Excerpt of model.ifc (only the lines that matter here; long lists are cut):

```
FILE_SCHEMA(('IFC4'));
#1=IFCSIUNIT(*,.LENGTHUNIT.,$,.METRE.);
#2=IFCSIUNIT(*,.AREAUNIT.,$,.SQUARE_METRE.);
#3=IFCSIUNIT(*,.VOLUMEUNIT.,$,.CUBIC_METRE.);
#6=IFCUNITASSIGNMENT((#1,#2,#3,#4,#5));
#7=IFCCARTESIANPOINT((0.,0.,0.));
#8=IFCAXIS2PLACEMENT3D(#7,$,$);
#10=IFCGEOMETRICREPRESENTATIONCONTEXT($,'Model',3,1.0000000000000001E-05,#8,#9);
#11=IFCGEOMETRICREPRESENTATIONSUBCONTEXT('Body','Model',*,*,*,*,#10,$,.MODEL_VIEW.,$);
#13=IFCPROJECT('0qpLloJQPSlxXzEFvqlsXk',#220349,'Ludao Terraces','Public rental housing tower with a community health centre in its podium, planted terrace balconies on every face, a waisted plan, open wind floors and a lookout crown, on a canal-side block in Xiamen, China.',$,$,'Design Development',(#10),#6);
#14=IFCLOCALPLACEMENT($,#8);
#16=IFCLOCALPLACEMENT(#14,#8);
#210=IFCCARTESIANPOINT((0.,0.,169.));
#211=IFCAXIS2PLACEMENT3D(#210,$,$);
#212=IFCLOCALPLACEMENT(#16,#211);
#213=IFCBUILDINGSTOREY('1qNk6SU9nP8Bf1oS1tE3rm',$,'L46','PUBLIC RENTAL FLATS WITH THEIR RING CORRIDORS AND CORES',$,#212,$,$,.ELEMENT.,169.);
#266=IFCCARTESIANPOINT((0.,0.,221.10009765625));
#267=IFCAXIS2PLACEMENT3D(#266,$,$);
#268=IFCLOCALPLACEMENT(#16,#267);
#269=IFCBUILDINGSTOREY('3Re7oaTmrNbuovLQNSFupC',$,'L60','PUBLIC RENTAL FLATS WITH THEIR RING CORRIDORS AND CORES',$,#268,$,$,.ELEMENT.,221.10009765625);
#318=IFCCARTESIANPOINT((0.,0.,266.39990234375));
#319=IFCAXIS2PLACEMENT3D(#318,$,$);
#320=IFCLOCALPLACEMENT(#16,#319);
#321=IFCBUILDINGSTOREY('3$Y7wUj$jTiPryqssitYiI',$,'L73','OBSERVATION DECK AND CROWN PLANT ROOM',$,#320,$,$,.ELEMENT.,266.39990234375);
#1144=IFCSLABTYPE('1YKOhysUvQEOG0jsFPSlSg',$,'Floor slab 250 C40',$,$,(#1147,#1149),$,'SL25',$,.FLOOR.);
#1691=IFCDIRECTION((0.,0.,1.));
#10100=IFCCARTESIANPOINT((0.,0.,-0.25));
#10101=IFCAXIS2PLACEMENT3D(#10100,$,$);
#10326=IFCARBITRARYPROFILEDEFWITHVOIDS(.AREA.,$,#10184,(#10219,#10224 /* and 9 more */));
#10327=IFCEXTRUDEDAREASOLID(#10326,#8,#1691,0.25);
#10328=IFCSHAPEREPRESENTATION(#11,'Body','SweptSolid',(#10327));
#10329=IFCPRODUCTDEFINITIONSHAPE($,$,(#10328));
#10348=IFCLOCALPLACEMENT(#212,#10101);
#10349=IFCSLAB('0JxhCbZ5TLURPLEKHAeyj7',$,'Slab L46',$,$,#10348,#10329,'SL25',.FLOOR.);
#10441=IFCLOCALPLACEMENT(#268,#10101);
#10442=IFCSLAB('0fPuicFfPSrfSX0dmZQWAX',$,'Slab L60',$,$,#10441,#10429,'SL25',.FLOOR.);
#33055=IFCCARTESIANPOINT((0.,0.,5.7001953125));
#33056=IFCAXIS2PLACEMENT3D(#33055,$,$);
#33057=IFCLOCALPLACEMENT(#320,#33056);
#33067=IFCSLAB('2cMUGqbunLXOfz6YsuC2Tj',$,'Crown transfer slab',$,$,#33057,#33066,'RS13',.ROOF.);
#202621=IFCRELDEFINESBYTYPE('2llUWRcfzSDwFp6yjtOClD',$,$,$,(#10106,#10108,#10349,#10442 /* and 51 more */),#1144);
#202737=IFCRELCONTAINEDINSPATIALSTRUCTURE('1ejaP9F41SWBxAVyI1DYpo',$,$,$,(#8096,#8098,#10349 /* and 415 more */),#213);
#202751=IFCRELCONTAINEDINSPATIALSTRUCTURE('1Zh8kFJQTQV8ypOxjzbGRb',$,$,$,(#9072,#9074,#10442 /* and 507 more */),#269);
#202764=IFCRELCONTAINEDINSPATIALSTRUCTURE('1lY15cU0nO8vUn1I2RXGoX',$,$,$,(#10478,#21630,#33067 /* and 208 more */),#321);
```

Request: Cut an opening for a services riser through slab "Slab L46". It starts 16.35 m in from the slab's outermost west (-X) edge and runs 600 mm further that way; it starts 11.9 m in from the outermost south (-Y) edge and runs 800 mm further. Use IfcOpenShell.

```python
import numpy as np
import ifcopenshell
import ifcopenshell.api.feature
import ifcopenshell.api.geometry
import ifcopenshell.api.root
import ifcopenshell.geom
import ifcopenshell.util.placement
import ifcopenshell.util.representation
import ifcopenshell.util.shape
import ifcopenshell.util.unit

model = ifcopenshell.open("model.ifc")
unit_scale = ifcopenshell.util.unit.calculate_unit_scale(model)
settings = ifcopenshell.geom.settings()


def volume(element):
    """Net volume in cubic metres, openings subtracted."""
    shape = ifcopenshell.geom.create_shape(settings, element)
    return ifcopenshell.util.shape.get_volume(shape.geometry)


slab = model.by_guid("0JxhCbZ5TLURPLEKHAeyj7")
before = volume(slab)

# Extent in the slab's own axes, in metres. The edges named are its -X and -Y sides.
slab_shape = ifcopenshell.geom.create_shape(settings, slab)
vertices = ifcopenshell.util.shape.get_vertices(slab_shape.geometry)
x_min, y_min, bottom = vertices.min(axis=0)
top = vertices[:, 2].max()

opening = ifcopenshell.api.root.create_entity(model, ifc_class="IfcOpeningElement", name="Services riser opening", predefined_type="OPENING")
context = ifcopenshell.util.representation.get_context(model, "Model", "Body", "MODEL_VIEW")
width, depth = 0.6, 0.8
outline = [(0.0, 0.0), (width, 0.0), (width, depth), (0.0, depth), (0.0, 0.0)]
# Overshoot both faces by 50 mm so the cut is clean.
shape = ifcopenshell.api.geometry.add_slab_representation(
    model, context=context, depth=top - bottom + 0.1, polyline=outline
)
ifcopenshell.api.geometry.assign_representation(model, product=opening, representation=shape)

matrix = ifcopenshell.util.placement.get_local_placement(slab.ObjectPlacement)
matrix[:, 3] = matrix @ np.append(np.array([x_min + 16.35, y_min + 11.9, bottom - 0.05]) / unit_scale, 1.0)
ifcopenshell.api.geometry.edit_object_placement(model, product=opening, matrix=matrix, is_si=False)
ifcopenshell.api.feature.add_feature(model, feature=opening, element=slab)

after = volume(slab)

print(f"slab volume {before:.3f} -> {after:.3f} m3")

model.write("model_v2.ifc")
```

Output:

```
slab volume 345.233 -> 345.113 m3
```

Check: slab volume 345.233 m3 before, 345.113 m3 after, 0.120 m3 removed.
